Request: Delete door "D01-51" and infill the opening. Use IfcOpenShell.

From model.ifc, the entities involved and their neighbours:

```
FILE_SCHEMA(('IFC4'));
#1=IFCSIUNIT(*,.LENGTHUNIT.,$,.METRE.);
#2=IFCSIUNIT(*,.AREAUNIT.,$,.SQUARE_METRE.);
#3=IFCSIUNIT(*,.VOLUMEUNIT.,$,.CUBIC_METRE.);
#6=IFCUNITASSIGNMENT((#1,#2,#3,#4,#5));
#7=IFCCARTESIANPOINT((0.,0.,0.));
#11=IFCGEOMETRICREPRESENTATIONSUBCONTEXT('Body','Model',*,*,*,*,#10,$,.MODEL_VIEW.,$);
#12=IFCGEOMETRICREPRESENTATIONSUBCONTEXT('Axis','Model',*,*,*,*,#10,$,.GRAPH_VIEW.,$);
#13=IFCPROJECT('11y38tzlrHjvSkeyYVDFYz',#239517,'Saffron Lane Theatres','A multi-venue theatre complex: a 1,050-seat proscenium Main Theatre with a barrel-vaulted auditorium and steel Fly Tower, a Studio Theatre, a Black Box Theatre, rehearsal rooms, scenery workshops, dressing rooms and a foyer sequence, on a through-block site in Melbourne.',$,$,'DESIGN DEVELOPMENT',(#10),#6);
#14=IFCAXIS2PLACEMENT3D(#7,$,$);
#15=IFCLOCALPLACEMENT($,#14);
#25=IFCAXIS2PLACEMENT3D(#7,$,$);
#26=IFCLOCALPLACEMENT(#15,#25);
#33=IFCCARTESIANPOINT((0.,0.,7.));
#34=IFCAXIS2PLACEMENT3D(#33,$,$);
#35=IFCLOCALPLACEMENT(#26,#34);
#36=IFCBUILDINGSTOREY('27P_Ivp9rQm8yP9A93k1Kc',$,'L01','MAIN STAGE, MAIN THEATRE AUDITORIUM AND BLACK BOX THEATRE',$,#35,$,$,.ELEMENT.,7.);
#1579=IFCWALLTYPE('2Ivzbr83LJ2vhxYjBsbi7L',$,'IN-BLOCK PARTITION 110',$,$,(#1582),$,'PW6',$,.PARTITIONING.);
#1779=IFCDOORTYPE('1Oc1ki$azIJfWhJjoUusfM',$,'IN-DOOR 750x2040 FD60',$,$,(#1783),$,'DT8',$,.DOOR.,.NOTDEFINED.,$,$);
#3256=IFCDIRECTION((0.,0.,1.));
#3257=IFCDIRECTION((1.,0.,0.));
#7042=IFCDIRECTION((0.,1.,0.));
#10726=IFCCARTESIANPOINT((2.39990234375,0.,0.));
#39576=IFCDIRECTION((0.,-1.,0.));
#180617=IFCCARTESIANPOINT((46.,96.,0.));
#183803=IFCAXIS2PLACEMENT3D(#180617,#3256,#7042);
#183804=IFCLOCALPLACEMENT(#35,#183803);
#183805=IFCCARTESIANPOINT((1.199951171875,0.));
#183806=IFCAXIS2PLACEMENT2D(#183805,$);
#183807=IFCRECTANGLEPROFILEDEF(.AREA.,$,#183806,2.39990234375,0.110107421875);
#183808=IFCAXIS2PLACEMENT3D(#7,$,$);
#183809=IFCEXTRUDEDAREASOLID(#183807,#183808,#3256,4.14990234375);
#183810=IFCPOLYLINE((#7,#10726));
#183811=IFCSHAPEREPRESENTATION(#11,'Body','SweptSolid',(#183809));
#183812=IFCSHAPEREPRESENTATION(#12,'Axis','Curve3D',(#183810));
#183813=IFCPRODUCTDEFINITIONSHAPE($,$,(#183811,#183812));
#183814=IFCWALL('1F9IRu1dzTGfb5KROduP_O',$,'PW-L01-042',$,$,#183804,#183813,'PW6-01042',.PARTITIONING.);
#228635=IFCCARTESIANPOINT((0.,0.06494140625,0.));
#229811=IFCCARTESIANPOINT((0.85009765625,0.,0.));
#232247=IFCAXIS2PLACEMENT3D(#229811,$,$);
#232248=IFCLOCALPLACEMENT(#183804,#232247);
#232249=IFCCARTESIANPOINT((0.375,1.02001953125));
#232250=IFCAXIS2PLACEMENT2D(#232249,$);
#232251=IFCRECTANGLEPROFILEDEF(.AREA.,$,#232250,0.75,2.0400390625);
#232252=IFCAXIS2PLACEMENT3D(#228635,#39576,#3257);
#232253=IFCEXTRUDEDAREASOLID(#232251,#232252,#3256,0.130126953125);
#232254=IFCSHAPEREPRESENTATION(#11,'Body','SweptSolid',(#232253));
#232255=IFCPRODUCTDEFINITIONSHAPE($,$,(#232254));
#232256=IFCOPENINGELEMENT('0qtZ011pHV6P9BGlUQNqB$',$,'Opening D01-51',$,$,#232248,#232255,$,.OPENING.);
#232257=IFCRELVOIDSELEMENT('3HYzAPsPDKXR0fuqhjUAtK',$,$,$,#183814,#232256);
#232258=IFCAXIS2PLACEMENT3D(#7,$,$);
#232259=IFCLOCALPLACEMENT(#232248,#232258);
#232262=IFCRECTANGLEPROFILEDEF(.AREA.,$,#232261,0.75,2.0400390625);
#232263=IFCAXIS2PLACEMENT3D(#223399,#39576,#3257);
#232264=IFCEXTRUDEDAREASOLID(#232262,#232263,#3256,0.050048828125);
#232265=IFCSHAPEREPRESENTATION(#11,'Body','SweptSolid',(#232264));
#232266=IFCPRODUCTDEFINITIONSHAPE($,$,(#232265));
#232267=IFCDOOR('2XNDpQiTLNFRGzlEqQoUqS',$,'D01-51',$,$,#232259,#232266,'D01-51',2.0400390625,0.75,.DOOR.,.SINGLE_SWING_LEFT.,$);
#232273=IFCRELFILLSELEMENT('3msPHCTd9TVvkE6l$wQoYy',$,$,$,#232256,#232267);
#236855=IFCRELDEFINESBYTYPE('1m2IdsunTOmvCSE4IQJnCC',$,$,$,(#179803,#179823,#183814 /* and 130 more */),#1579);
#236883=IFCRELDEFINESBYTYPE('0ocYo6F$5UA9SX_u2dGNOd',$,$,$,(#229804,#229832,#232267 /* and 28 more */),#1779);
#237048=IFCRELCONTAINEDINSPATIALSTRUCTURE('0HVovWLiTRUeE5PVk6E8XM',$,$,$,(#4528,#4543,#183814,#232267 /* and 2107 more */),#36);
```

```python
import ifcopenshell
import ifcopenshell.api.feature
import ifcopenshell.api.root
import ifcopenshell.geom
import ifcopenshell.util.shape

model = ifcopenshell.open("model.ifc")
settings = ifcopenshell.geom.settings()


def volume(element):
    """Net volume in cubic metres, openings subtracted."""
    shape = ifcopenshell.geom.create_shape(settings, element)
    return ifcopenshell.util.shape.get_volume(shape.geometry)


door = model.by_id(232267)
opening = door.FillsVoids[0].RelatingOpeningElement
wall = opening.VoidsElements[0].RelatingBuildingElement
before = volume(wall)

ifcopenshell.api.root.remove_product(model, product=door)
ifcopenshell.api.feature.remove_feature(model, feature=opening)

after = volume(wall)

print(f"wall volume {before:.3f} -> {after:.3f} m3")

model.write("model-out.ifc")
```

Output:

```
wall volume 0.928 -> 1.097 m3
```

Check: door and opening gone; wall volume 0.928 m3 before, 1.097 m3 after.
